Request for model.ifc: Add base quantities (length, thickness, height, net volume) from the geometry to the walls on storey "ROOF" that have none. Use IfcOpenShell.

First a look at what the model holds.

```python
import ifcopenshell
import ifcopenshell.util.element
import ifcopenshell.util.unit

model = ifcopenshell.open("model.ifc")
print(model.schema)
for unit_type in ("LENGTHUNIT", "AREAUNIT", "VOLUMEUNIT"):
    print(unit_type, ifcopenshell.util.unit.calculate_unit_scale(model, unit_type))
storey = next(s for s in model.by_type("IfcBuildingStorey") if s.Name == "ROOF")
walls = [e for e in ifcopenshell.util.element.get_decomposition(storey) if e.is_a("IfcWall")]
for e in sorted(walls, key=lambda e: e.id()):
    print(e.id(), e.is_a(), e.Name, list(ifcopenshell.util.element.get_psets(e, qtos_only=True)), sep=" | ")
```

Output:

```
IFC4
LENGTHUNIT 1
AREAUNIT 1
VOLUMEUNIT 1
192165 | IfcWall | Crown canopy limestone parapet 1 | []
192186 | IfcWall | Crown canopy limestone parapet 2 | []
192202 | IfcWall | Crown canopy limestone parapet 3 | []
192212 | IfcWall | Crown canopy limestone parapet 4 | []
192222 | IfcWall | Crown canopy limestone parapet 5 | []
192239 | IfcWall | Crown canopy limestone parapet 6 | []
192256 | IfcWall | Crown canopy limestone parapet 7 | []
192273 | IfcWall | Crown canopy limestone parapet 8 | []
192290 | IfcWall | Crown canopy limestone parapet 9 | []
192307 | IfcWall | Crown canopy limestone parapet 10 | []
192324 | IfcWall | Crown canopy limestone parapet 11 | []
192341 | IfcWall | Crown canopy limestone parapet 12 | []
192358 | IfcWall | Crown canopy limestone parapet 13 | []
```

```python
import ifcopenshell
import ifcopenshell.api.pset
import ifcopenshell.geom
import ifcopenshell.util.element
import ifcopenshell.util.shape
import ifcopenshell.util.unit

model = ifcopenshell.open("model.ifc")
unit_scale = ifcopenshell.util.unit.calculate_unit_scale(model)
volume_scale = ifcopenshell.util.unit.calculate_unit_scale(model, "VOLUMEUNIT")
settings = ifcopenshell.geom.settings()

storey = next(s for s in model.by_type("IfcBuildingStorey") if s.Name == "ROOF")
walls = [e for e in ifcopenshell.util.element.get_decomposition(storey) if e.is_a("IfcWall")]

for e in sorted(walls, key=lambda e: e.id()):
    if ifcopenshell.util.element.get_psets(e, qtos_only=True, should_inherit=False):
        continue
    # Geometry comes back in metres, in the element's own axes.
    shape = ifcopenshell.geom.create_shape(settings, e)
    values = {
        "Length": ifcopenshell.util.shape.get_x(shape.geometry) / unit_scale,
        "Width": ifcopenshell.util.shape.get_y(shape.geometry) / unit_scale,
        "Height": ifcopenshell.util.shape.get_z(shape.geometry) / unit_scale,
        "NetVolume": ifcopenshell.util.shape.get_volume(shape.geometry) / volume_scale,
    }
    qto = ifcopenshell.api.pset.add_qto(model, product=e, name="Qto_WallBaseQuantities")
    ifcopenshell.api.pset.edit_qto(model, qto=qto, properties=values)
    print(e.id(), {k: round(v, 3) for k, v in values.items()})

model.write("model-out.ifc")
```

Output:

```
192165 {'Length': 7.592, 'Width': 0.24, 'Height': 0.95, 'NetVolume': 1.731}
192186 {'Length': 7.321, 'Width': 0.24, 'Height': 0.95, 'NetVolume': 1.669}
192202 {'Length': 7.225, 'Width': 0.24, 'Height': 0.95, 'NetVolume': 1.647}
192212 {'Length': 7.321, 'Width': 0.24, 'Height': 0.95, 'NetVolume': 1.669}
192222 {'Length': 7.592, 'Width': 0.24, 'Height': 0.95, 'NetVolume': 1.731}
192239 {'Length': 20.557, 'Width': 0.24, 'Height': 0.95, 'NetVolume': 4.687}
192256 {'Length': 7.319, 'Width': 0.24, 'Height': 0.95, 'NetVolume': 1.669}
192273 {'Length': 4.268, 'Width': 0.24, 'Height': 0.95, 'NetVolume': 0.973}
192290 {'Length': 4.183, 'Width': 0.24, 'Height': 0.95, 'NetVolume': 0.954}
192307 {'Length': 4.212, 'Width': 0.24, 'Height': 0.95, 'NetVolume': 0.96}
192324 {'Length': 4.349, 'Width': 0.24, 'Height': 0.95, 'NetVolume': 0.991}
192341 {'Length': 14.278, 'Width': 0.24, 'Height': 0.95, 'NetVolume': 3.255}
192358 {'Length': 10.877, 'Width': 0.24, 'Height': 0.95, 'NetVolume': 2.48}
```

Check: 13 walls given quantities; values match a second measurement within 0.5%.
